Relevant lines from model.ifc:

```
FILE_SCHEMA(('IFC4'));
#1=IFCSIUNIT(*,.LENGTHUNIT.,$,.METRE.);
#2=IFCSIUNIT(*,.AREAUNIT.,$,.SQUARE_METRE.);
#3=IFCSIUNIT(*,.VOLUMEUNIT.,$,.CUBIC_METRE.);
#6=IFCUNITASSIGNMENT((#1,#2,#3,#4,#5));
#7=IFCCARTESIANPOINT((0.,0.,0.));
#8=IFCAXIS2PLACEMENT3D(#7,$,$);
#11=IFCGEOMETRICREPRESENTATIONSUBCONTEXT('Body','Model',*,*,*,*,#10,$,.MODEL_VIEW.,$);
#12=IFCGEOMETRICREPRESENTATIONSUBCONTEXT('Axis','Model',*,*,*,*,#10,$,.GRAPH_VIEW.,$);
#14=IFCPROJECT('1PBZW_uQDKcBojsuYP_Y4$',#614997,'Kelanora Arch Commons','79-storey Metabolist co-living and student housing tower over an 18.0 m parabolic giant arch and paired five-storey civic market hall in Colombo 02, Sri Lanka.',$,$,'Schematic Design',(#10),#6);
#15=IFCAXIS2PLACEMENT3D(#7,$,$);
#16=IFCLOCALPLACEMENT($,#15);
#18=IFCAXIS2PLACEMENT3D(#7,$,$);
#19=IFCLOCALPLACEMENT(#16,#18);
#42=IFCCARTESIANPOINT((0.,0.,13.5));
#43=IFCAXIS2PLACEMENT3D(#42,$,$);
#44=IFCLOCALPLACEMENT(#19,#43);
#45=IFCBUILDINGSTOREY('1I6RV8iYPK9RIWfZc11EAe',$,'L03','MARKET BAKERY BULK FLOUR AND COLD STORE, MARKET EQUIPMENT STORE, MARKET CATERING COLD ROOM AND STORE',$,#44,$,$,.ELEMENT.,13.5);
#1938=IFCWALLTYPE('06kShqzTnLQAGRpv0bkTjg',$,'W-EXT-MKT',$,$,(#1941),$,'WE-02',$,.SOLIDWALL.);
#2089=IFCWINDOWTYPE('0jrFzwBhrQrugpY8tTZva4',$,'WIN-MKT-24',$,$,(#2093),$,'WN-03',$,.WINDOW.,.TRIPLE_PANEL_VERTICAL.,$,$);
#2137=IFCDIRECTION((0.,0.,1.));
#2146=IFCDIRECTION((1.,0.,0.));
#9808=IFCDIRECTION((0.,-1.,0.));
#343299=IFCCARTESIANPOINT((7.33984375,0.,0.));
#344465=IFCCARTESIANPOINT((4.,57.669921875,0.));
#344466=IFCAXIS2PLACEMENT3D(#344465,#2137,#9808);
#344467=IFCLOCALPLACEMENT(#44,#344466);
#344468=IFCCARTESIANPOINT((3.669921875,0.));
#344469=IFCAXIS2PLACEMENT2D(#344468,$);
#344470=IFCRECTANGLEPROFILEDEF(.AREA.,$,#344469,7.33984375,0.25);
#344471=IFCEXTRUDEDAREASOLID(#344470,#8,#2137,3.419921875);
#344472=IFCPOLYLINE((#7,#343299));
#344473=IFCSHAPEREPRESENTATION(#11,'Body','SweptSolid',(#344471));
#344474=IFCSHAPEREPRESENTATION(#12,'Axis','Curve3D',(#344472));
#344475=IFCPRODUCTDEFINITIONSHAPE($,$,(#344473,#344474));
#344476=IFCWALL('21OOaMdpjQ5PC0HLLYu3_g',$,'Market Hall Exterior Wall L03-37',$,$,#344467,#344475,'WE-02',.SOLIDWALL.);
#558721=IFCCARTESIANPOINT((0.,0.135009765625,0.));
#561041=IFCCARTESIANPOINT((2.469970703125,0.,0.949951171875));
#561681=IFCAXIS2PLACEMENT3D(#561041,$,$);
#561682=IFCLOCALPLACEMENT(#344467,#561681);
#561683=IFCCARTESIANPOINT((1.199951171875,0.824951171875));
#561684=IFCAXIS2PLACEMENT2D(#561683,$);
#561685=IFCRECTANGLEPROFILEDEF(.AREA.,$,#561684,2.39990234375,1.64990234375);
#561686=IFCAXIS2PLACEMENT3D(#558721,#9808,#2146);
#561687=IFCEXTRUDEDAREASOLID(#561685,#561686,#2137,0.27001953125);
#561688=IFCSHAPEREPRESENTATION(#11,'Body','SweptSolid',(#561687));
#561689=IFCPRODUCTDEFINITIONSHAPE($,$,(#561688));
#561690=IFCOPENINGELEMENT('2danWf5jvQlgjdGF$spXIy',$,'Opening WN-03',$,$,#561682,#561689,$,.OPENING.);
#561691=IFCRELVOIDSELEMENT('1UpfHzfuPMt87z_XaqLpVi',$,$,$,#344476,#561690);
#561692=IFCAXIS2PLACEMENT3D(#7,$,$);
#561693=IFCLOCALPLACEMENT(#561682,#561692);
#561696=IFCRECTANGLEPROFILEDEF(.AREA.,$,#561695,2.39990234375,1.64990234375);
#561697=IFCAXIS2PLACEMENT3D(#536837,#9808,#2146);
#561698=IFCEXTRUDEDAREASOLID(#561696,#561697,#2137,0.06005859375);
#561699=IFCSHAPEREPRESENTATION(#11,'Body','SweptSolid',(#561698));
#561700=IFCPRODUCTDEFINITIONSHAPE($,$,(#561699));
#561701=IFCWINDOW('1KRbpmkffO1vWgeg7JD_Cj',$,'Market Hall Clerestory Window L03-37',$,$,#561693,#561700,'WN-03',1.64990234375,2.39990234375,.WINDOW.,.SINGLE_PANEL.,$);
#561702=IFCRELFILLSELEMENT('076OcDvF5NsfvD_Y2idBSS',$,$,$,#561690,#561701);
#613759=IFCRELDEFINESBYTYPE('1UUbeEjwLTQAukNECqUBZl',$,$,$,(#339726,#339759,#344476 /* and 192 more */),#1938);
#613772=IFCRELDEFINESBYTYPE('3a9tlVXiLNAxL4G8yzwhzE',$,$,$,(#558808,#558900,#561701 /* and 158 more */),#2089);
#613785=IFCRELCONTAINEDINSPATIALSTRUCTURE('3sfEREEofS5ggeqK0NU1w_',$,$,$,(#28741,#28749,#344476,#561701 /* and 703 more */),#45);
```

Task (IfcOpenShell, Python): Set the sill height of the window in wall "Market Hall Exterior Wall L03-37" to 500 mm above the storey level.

```python
import numpy as np
import ifcopenshell
import ifcopenshell.api.geometry
import ifcopenshell.geom
import ifcopenshell.util.element
import ifcopenshell.util.placement
import ifcopenshell.util.shape
import ifcopenshell.util.unit

model = ifcopenshell.open("model.ifc")
unit_scale = ifcopenshell.util.unit.calculate_unit_scale(model)

window = model.by_guid("1KRbpmkffO1vWgeg7JD_Cj")
opening = window.FillsVoids[0].RelatingOpeningElement
storey = ifcopenshell.util.element.get_container(window, ifc_class="IfcBuildingStorey")
level = ifcopenshell.util.placement.get_local_placement(storey.ObjectPlacement)[2, 3]

# The opening's origin need not be at the sill, so measure its lowest point.
shape = ifcopenshell.geom.create_shape(ifcopenshell.geom.settings(), opening)
bottom = ifcopenshell.util.shape.get_shape_bottom_elevation(shape, shape.geometry) / unit_scale
dz = level + 0.5 / unit_scale - bottom

shift = np.array([0.0, 0.0, dz])
# The window is placed relative to its opening, so it follows when the opening moves.
matrix = ifcopenshell.util.placement.get_local_placement(opening.ObjectPlacement)
matrix[:3, 3] += shift
ifcopenshell.api.geometry.edit_object_placement(
    model, product=opening, matrix=matrix, is_si=False, should_transform_children=True
)

print(f"moved by {dz * unit_scale:+.3f} m")

model.write("model_rev.ifc")
```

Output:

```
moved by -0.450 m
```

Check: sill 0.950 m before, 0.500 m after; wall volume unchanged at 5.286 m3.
